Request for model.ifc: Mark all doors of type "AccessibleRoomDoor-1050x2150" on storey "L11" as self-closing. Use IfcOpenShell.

First a look at what the model holds.

```python
import ifcopenshell
import ifcopenshell.util.element

model = ifcopenshell.open("model.ifc")
print(model.schema)
storey = next(s for s in model.by_type("IfcBuildingStorey") if s.Name == "L11")
doors = [e for e in ifcopenshell.util.element.get_decomposition(storey) if e.is_a("IfcDoor")]
seen = {}
for e in doors:
    element_type = ifcopenshell.util.element.get_type(e)
    key = (element_type.Name if element_type != e and element_type else None, ifcopenshell.util.element.get_pset(e, "Pset_DoorCommon", "SelfClosing"))
    seen[key] = seen.get(key, 0) + 1
for (name, value), count in sorted(seen.items(), key=str):
    print(count, "x", name, "|", value)
```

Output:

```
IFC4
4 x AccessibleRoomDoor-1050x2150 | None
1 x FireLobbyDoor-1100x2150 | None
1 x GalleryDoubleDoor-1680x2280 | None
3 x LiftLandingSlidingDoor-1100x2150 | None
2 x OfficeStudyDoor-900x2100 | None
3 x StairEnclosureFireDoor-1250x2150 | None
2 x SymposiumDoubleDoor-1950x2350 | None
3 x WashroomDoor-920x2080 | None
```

```python
import ifcopenshell
import ifcopenshell.api.pset
import ifcopenshell.util.element

model = ifcopenshell.open("model.ifc")

storey = next(s for s in model.by_type("IfcBuildingStorey") if s.Name == "L11")
doors = [e for e in ifcopenshell.util.element.get_decomposition(storey) if e.is_a("IfcDoor")]

count = 0
for e in doors:
    element_type = ifcopenshell.util.element.get_type(e)
    if element_type in (None, e) or element_type.Name != "AccessibleRoomDoor-1050x2150":
        continue
    # add_pset returns the element's existing set when there is one.
    pset = ifcopenshell.api.pset.add_pset(model, product=e, name="Pset_DoorCommon")
    ifcopenshell.api.pset.edit_pset(model, pset=pset, properties={"SelfClosing": True})
    count += 1

print(count, "doors updated")

model.write("model_rev.ifc")
```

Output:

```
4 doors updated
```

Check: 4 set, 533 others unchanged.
